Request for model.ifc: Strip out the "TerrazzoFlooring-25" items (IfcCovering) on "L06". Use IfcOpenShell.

First a look at what the model holds.

```python
import ifcopenshell
import ifcopenshell.util.element

model = ifcopenshell.open("model.ifc")
print(model.schema)
storey = next(s for s in model.by_type("IfcBuildingStorey") if s.Name == "L06")
coverings = [e for e in ifcopenshell.util.element.get_decomposition(storey) if e.is_a("IfcCovering")]
seen = {}
for e in coverings:
    element_type = ifcopenshell.util.element.get_type(e)
    name = element_type.Name if element_type not in (None, e) else None
    seen[name] = seen.get(name, 0) + 1
for name, count in sorted(seen.items(), key=str):
    print(count, "x", name)
```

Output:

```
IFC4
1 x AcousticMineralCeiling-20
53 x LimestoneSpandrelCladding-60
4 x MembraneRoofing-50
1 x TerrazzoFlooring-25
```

```python
import ifcopenshell
import ifcopenshell.api.root
import ifcopenshell.util.element

model = ifcopenshell.open("model.ifc")

storey = next(s for s in model.by_type("IfcBuildingStorey") if s.Name == "L06")
coverings = [e for e in ifcopenshell.util.element.get_decomposition(storey) if e.is_a("IfcCovering")]
targets = [e for e in coverings if (t := ifcopenshell.util.element.get_type(e)) not in (None, e) and t.Name == "TerrazzoFlooring-25"]

for e in targets:
    ifcopenshell.api.root.remove_product(model, product=e)
print(len(targets), "removed")

model.write("model_rev.ifc")
```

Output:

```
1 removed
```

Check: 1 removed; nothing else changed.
